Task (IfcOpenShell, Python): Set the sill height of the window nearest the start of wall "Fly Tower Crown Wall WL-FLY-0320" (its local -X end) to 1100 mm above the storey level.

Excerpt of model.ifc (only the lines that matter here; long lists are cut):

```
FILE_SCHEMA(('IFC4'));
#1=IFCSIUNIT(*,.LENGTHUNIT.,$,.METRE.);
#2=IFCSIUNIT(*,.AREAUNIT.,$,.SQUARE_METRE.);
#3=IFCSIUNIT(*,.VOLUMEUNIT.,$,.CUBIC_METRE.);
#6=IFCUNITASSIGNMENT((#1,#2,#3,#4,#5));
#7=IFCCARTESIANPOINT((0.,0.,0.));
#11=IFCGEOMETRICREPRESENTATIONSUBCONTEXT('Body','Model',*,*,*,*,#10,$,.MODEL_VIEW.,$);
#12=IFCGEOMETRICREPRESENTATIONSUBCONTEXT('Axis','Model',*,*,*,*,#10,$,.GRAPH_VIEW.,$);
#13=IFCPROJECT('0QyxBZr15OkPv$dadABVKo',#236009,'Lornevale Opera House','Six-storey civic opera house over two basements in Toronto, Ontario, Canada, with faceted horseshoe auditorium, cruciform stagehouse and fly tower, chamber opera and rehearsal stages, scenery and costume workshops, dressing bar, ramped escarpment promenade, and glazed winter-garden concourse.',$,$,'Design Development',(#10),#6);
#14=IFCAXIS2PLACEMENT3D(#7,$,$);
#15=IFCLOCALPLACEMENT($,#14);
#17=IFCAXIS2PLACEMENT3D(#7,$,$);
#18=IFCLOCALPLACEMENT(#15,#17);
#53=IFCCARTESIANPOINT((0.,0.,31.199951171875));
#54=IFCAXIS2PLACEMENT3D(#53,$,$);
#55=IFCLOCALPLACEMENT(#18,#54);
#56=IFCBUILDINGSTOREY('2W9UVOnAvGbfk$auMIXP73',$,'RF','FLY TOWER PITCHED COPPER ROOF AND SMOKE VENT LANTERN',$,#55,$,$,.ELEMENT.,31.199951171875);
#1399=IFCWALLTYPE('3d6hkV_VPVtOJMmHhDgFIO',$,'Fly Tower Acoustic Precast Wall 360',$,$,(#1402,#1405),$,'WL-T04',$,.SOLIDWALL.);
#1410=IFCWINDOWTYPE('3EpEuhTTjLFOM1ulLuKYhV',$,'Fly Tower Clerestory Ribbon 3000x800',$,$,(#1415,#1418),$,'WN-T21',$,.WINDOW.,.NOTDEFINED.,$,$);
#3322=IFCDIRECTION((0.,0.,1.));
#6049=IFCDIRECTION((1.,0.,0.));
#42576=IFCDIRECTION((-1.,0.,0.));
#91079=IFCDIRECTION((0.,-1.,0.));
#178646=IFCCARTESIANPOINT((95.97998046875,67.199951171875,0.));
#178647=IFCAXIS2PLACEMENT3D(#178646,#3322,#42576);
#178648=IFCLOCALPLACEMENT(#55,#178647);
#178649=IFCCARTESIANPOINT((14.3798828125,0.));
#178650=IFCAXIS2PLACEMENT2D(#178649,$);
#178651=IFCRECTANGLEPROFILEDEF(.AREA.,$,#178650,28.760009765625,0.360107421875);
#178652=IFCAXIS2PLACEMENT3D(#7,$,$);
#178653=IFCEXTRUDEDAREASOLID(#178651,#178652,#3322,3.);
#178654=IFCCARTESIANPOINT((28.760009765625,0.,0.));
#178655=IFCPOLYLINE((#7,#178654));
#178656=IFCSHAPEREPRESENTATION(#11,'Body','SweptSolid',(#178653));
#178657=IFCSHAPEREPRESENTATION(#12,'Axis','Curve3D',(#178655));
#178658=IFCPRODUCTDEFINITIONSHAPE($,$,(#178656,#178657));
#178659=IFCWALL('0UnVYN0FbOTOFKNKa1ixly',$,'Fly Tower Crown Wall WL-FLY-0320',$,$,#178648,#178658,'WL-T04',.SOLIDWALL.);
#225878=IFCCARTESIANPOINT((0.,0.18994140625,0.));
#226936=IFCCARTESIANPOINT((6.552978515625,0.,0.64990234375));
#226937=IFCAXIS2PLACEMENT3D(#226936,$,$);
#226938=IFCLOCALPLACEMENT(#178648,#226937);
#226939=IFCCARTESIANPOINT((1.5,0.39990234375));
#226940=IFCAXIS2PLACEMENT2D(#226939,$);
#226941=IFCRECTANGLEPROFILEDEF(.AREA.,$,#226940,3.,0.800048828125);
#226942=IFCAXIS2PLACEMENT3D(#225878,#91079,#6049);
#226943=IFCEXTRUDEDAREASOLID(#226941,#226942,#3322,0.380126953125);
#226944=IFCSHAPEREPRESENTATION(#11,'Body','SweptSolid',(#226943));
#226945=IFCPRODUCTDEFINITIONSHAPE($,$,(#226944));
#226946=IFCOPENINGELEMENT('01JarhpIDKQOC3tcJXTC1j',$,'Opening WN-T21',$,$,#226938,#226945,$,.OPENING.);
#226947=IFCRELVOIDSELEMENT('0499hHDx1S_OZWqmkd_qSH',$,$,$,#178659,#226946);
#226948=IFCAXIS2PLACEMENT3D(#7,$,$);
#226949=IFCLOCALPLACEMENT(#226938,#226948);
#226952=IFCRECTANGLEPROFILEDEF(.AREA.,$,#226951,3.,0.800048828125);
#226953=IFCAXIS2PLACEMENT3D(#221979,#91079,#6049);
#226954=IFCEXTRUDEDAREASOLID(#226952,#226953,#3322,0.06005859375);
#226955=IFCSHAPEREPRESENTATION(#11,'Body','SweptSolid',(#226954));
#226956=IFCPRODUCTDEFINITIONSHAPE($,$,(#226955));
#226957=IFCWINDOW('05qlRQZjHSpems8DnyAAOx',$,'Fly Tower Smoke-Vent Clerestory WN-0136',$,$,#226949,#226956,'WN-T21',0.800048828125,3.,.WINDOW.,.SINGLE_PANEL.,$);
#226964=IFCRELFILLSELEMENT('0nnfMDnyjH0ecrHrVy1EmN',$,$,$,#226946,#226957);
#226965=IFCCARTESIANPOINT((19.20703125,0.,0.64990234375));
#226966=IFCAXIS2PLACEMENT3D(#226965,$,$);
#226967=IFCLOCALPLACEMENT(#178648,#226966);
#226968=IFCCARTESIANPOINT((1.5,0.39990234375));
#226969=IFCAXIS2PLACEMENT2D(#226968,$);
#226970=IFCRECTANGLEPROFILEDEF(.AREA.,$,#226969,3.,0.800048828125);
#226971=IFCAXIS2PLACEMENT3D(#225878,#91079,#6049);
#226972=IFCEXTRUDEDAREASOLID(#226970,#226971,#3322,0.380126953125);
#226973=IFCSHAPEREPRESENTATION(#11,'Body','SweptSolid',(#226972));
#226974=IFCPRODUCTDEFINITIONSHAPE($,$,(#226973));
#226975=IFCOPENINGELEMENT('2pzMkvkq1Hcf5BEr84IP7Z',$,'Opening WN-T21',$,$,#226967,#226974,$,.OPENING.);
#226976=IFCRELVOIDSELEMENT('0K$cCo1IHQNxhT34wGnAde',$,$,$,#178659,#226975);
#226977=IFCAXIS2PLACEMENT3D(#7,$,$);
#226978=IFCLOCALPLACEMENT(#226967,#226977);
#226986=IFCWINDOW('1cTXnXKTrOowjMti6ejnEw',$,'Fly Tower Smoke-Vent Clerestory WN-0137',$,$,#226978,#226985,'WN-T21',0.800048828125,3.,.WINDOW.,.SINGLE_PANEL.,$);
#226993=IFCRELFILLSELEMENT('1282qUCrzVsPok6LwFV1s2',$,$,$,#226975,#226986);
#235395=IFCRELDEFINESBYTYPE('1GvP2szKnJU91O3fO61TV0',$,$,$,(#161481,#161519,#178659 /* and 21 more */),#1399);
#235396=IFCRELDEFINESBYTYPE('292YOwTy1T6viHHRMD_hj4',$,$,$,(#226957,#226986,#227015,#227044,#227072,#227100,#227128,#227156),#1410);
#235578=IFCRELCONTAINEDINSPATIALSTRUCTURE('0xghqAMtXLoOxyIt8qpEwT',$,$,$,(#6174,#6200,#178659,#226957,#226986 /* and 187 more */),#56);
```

```python
import numpy as np
import ifcopenshell
import ifcopenshell.api.geometry
import ifcopenshell.geom
import ifcopenshell.util.element
import ifcopenshell.util.placement
import ifcopenshell.util.shape
import ifcopenshell.util.unit

model = ifcopenshell.open("model.ifc")
unit_scale = ifcopenshell.util.unit.calculate_unit_scale(model)

window = model.by_id(226957)
opening = window.FillsVoids[0].RelatingOpeningElement
storey = ifcopenshell.util.element.get_container(window, ifc_class="IfcBuildingStorey")
level = ifcopenshell.util.placement.get_local_placement(storey.ObjectPlacement)[2, 3]

# The opening's origin need not be at the sill, so measure its lowest point.
shape = ifcopenshell.geom.create_shape(ifcopenshell.geom.settings(), opening)
bottom = ifcopenshell.util.shape.get_shape_bottom_elevation(shape, shape.geometry) / unit_scale
dz = level + 1.1 - bottom

shift = np.array([0.0, 0.0, dz])
# The window is placed relative to its opening, so it follows when the opening moves.
matrix = ifcopenshell.util.placement.get_local_placement(opening.ObjectPlacement)
matrix[:3, 3] += shift
ifcopenshell.api.geometry.edit_object_placement(
    model, product=opening, matrix=matrix, is_si=False, should_transform_children=True
)

print(f"moved by {dz * unit_scale:+.3f} m")

model.write("model_edited.ifc")
```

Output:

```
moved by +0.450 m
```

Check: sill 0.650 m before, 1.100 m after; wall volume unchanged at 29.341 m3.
